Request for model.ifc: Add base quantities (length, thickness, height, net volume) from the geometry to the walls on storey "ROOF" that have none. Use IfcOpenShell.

First a look at what the model holds.

```python
import ifcopenshell
import ifcopenshell.util.element
import ifcopenshell.util.unit

model = ifcopenshell.open("model.ifc")
print(model.schema)
for unit_type in ("LENGTHUNIT", "AREAUNIT", "VOLUMEUNIT"):
    print(unit_type, ifcopenshell.util.unit.calculate_unit_scale(model, unit_type))
storey = next(s for s in model.by_type("IfcBuildingStorey") if s.Name == "ROOF")
walls = [e for e in ifcopenshell.util.element.get_decomposition(storey) if e.is_a("IfcWall")]
for e in sorted(walls, key=lambda e: e.id()):
    print(e.id(), e.is_a(), e.Name, list(ifcopenshell.util.element.get_psets(e, qtos_only=True)), sep=" | ")
```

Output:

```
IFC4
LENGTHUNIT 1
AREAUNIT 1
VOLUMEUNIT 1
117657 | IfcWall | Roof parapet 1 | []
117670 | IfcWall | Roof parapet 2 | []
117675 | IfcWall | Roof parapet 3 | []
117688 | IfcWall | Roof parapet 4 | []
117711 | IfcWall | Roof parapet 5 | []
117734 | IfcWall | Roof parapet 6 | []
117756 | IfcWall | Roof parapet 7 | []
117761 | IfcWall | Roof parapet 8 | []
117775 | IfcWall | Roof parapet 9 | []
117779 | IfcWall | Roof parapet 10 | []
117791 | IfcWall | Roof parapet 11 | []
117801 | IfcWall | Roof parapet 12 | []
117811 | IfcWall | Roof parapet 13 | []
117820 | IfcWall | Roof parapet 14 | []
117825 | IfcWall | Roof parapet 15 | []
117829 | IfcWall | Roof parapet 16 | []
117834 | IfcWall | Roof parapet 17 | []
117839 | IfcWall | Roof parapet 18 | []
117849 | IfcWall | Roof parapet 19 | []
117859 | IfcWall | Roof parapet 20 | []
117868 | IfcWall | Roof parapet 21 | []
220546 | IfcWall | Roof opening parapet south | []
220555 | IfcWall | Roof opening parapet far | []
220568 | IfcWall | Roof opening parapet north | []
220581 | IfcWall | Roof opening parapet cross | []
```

```python
import ifcopenshell
import ifcopenshell.api.pset
import ifcopenshell.geom
import ifcopenshell.util.element
import ifcopenshell.util.shape
import ifcopenshell.util.unit

model = ifcopenshell.open("model.ifc")
unit_scale = ifcopenshell.util.unit.calculate_unit_scale(model)
volume_scale = ifcopenshell.util.unit.calculate_unit_scale(model, "VOLUMEUNIT")
settings = ifcopenshell.geom.settings()

storey = next(s for s in model.by_type("IfcBuildingStorey") if s.Name == "ROOF")
walls = [e for e in ifcopenshell.util.element.get_decomposition(storey) if e.is_a("IfcWall")]

for e in sorted(walls, key=lambda e: e.id()):
    if ifcopenshell.util.element.get_psets(e, qtos_only=True, should_inherit=False):
        continue
    # Geometry comes back in metres, in the element's own axes.
    shape = ifcopenshell.geom.create_shape(settings, e)
    values = {
        "Length": ifcopenshell.util.shape.get_x(shape.geometry) / unit_scale,
        "Width": ifcopenshell.util.shape.get_y(shape.geometry) / unit_scale,
        "Height": ifcopenshell.util.shape.get_z(shape.geometry) / unit_scale,
        "NetVolume": ifcopenshell.util.shape.get_volume(shape.geometry) / volume_scale,
    }
    qto = ifcopenshell.api.pset.add_qto(model, product=e, name="Qto_WallBaseQuantities")
    ifcopenshell.api.pset.edit_qto(model, qto=qto, properties=values)
    print(e.id(), {k: round(v, 3) for k, v in values.items()})

model.write("model_edited.ifc")
```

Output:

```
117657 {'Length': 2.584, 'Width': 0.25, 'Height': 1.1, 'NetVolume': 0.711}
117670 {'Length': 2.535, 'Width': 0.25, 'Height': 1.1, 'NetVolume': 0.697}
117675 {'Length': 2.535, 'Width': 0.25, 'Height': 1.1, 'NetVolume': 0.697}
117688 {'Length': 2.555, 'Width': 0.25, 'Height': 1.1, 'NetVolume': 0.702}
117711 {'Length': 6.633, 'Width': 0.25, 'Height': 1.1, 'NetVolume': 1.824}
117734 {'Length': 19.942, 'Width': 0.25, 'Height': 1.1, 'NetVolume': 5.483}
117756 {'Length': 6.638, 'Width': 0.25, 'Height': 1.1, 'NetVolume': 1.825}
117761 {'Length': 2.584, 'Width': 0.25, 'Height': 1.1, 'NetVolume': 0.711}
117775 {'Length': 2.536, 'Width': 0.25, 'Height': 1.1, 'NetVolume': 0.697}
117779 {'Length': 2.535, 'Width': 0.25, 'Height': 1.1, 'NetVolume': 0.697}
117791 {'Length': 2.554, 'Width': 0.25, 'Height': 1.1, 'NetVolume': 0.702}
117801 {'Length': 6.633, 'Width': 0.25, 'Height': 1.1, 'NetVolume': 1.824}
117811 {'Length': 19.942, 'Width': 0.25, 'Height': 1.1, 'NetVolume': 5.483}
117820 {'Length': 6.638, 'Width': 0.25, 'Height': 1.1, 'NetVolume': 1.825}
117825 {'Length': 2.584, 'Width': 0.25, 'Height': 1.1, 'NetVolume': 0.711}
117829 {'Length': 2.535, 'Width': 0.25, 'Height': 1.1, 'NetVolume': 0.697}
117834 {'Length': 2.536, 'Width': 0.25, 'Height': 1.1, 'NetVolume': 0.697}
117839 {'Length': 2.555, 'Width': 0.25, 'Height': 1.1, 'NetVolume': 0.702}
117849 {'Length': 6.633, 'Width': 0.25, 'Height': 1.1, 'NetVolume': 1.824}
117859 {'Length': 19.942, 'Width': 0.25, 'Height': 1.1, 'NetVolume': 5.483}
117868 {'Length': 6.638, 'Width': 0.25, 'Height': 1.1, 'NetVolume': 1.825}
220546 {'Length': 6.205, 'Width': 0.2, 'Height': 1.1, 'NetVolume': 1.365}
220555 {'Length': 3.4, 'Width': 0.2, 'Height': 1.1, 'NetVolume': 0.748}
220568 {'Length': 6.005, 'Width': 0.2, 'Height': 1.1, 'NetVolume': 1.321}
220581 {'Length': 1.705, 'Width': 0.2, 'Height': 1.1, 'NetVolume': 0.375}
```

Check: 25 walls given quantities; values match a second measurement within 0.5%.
